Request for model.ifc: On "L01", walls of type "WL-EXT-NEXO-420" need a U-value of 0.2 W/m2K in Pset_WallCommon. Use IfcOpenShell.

First a look at what the model holds.

```python
import ifcopenshell
import ifcopenshell.util.element

model = ifcopenshell.open("model.ifc")
print(model.schema)
storey = next(s for s in model.by_type("IfcBuildingStorey") if s.Name == "L01")
walls = [e for e in ifcopenshell.util.element.get_decomposition(storey) if e.is_a("IfcWall")]
seen = {}
for e in walls:
    element_type = ifcopenshell.util.element.get_type(e)
    key = (element_type.Name if element_type != e and element_type else None, ifcopenshell.util.element.get_pset(e, "Pset_WallCommon", "ThermalTransmittance"))
    seen[key] = seen.get(key, 0) + 1
for (name, value), count in sorted(seen.items(), key=str):
    print(count, "x", name, "|", value)
```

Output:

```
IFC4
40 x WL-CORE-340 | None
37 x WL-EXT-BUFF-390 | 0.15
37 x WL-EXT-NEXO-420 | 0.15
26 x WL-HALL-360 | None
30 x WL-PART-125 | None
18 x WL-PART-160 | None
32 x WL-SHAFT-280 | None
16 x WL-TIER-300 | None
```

```python
import ifcopenshell
import ifcopenshell.api.pset
import ifcopenshell.util.element

model = ifcopenshell.open("model.ifc")

storey = next(s for s in model.by_type("IfcBuildingStorey") if s.Name == "L01")
walls = [e for e in ifcopenshell.util.element.get_decomposition(storey) if e.is_a("IfcWall")]

count = 0
for e in walls:
    element_type = ifcopenshell.util.element.get_type(e)
    if element_type in (None, e) or element_type.Name != "WL-EXT-NEXO-420":
        continue
    # add_pset returns the element's existing set when there is one.
    pset = ifcopenshell.api.pset.add_pset(model, product=e, name="Pset_WallCommon")
    ifcopenshell.api.pset.edit_pset(model, pset=pset, properties={"ThermalTransmittance": 0.2})
    count += 1

print(count, "walls updated")

model.write("model_rev.ifc")
```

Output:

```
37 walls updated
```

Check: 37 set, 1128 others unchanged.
